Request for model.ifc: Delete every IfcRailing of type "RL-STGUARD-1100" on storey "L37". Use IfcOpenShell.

First a look at what the model holds.

```python
import ifcopenshell
import ifcopenshell.util.element

model = ifcopenshell.open("model.ifc")
print(model.schema)
storey = next(s for s in model.by_type("IfcBuildingStorey") if s.Name == "L37")
railings = [e for e in ifcopenshell.util.element.get_decomposition(storey) if e.is_a("IfcRailing")]
seen = {}
for e in railings:
    element_type = ifcopenshell.util.element.get_type(e)
    name = element_type.Name if element_type not in (None, e) else None
    seen[name] = seen.get(name, 0) + 1
for name, count in sorted(seen.items(), key=str):
    print(count, "x", name)
```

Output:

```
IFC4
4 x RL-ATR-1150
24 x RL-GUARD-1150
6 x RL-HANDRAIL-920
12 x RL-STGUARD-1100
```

```python
import ifcopenshell
import ifcopenshell.api.root
import ifcopenshell.util.element

model = ifcopenshell.open("model.ifc")

storey = next(s for s in model.by_type("IfcBuildingStorey") if s.Name == "L37")
railings = [e for e in ifcopenshell.util.element.get_decomposition(storey) if e.is_a("IfcRailing")]
targets = [e for e in railings if (t := ifcopenshell.util.element.get_type(e)) not in (None, e) and t.Name == "RL-STGUARD-1100"]

for e in targets:
    ifcopenshell.api.root.remove_product(model, product=e)
print(len(targets), "removed")

model.write("model_updated.ifc")
```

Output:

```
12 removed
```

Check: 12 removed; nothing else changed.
